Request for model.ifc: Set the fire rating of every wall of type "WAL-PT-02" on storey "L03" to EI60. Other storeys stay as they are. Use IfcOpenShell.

First a look at what the model holds.

```python
import ifcopenshell
import ifcopenshell.util.element

model = ifcopenshell.open("model.ifc")
print(model.schema)
storey = next(s for s in model.by_type("IfcBuildingStorey") if s.Name == "L03")
walls = [e for e in ifcopenshell.util.element.get_decomposition(storey) if e.is_a("IfcWall")]
seen = {}
for e in walls:
    element_type = ifcopenshell.util.element.get_type(e)
    key = (element_type.Name if element_type != e and element_type else None, ifcopenshell.util.element.get_pset(e, "Pset_WallCommon", "FireRating"))
    seen[key] = seen.get(key, 0) + 1
for (name, value), count in sorted(seen.items(), key=str):
    print(count, "x", name, "|", value)
```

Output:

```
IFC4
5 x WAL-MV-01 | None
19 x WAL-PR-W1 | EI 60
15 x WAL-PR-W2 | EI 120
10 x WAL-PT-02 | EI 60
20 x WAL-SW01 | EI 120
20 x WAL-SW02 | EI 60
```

```python
import ifcopenshell
import ifcopenshell.api.pset
import ifcopenshell.util.element

model = ifcopenshell.open("model.ifc")

storey = next(s for s in model.by_type("IfcBuildingStorey") if s.Name == "L03")
walls = [e for e in ifcopenshell.util.element.get_decomposition(storey) if e.is_a("IfcWall")]

count = 0
for e in walls:
    element_type = ifcopenshell.util.element.get_type(e)
    if element_type in (None, e) or element_type.Name != "WAL-PT-02":
        continue
    # add_pset returns the element's existing set when there is one.
    pset = ifcopenshell.api.pset.add_pset(model, product=e, name="Pset_WallCommon")
    ifcopenshell.api.pset.edit_pset(model, pset=pset, properties={"FireRating": "EI60"})
    count += 1

print(count, "walls updated")

model.write("model-out.ifc")
```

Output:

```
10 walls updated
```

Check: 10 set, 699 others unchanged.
